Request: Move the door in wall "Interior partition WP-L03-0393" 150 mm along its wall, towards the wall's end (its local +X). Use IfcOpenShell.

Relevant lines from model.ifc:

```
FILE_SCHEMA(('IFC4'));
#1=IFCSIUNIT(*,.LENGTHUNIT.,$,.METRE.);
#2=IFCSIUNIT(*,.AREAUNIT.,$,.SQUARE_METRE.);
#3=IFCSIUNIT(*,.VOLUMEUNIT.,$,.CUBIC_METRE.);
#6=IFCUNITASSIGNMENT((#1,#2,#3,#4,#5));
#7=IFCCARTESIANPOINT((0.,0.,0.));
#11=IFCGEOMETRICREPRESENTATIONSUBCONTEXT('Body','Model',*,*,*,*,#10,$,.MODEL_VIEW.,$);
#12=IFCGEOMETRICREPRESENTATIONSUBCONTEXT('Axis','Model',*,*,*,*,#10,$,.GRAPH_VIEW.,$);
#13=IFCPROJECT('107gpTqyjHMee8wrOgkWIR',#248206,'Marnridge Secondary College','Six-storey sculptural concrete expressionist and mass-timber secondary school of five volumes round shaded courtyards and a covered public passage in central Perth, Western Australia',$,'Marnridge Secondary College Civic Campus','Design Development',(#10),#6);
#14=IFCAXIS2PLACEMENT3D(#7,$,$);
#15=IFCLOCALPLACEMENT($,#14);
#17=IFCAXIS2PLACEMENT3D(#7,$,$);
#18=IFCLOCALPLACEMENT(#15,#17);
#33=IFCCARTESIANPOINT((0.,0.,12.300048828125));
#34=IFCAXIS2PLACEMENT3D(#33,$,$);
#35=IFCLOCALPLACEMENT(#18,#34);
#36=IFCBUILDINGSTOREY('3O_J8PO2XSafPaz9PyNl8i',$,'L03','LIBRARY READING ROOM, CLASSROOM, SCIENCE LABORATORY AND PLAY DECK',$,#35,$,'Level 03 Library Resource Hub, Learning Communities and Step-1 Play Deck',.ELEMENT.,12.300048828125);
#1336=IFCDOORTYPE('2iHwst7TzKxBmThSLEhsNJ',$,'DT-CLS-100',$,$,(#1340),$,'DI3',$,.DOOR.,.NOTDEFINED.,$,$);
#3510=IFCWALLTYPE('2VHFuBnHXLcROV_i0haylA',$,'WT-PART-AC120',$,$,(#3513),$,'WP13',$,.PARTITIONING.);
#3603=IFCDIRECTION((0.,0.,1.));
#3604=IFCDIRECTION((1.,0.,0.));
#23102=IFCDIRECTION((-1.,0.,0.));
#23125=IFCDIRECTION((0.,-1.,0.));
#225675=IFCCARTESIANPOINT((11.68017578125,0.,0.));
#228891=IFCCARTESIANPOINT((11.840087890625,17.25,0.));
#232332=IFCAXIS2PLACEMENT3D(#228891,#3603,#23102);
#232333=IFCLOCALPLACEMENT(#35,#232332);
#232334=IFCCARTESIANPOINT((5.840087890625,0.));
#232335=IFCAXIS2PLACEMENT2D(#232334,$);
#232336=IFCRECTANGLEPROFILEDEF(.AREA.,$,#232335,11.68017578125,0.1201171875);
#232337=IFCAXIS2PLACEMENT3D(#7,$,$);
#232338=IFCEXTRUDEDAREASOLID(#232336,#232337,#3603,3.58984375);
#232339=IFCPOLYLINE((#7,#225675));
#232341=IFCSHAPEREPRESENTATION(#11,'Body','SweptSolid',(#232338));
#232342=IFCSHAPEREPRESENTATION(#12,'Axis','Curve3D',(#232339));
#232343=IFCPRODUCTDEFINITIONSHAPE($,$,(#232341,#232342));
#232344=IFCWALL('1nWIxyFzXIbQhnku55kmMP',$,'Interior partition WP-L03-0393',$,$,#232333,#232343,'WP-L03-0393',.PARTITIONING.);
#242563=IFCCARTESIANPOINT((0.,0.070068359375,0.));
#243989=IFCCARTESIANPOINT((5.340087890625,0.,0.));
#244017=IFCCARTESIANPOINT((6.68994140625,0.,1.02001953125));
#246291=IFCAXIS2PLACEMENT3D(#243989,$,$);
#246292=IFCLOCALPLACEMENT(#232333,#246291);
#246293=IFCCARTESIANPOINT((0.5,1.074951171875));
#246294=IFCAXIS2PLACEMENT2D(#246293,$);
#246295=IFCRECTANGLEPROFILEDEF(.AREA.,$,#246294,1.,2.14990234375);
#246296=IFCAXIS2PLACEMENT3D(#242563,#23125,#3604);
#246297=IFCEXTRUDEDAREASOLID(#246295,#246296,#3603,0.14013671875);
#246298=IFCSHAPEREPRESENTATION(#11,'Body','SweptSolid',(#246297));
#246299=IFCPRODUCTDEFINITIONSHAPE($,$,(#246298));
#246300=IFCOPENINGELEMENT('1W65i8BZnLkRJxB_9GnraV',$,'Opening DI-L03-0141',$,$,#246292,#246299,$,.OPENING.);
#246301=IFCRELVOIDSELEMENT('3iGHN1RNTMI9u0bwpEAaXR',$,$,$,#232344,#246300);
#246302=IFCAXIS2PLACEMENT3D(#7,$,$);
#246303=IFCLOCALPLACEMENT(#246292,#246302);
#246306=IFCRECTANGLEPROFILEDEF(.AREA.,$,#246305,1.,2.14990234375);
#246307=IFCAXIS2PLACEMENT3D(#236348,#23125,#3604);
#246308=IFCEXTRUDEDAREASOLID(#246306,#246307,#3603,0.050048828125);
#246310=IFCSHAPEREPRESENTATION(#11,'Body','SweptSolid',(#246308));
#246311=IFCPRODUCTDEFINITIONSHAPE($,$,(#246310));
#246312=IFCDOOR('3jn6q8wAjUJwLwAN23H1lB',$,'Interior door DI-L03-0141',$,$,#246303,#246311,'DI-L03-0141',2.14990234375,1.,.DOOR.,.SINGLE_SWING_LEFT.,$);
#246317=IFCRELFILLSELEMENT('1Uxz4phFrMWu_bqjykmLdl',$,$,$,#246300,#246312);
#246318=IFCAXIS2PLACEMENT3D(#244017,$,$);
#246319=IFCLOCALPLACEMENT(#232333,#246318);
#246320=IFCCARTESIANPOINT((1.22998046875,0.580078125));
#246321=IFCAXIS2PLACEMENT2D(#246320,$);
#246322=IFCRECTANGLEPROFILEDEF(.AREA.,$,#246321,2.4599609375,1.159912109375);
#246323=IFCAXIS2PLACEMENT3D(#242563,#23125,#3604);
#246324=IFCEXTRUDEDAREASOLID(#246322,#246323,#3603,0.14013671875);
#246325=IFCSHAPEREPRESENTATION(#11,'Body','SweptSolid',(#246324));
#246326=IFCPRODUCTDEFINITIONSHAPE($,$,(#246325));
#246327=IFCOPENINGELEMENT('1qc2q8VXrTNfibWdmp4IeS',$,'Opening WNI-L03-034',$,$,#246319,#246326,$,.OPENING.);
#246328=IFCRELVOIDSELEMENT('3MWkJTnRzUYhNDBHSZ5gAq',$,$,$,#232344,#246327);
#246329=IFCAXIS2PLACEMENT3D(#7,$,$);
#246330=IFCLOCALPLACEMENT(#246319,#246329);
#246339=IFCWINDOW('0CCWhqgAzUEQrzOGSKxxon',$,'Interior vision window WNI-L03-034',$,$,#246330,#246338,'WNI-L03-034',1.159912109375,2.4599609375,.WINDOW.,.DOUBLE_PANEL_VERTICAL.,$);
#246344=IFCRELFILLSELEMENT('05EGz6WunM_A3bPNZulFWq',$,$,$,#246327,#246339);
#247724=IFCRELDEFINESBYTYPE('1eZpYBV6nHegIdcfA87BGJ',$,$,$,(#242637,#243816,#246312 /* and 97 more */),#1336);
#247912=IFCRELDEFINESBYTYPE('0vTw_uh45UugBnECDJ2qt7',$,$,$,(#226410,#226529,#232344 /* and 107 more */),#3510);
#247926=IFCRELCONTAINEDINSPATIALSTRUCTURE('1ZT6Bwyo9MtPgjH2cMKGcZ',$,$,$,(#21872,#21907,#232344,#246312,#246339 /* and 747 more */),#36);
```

```python
import ifcopenshell
import ifcopenshell.api.geometry
import ifcopenshell.util.placement

model = ifcopenshell.open("model.ifc")

door = model.by_guid("3jn6q8wAjUJwLwAN23H1lB")
opening = door.FillsVoids[0].RelatingOpeningElement
wall = opening.VoidsElements[0].RelatingBuildingElement

wall_matrix = ifcopenshell.util.placement.get_local_placement(wall.ObjectPlacement)
shift = wall_matrix[:3, 0] * 0.15
before = ifcopenshell.util.placement.get_local_placement(door.ObjectPlacement)[:3, 3].copy()

# The door is placed relative to its opening, so it follows when the opening moves.
matrix = ifcopenshell.util.placement.get_local_placement(opening.ObjectPlacement)
matrix[:3, 3] += shift
ifcopenshell.api.geometry.edit_object_placement(
    model, product=opening, matrix=matrix, is_si=False, should_transform_children=True
)

after = ifcopenshell.util.placement.get_local_placement(door.ObjectPlacement)[:3, 3]
print("door moved by", (after - before).round(3) + 0.0)

model.write("model_v2.ifc")
```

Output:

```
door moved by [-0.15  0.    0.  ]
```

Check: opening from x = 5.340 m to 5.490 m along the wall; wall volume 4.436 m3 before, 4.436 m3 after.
